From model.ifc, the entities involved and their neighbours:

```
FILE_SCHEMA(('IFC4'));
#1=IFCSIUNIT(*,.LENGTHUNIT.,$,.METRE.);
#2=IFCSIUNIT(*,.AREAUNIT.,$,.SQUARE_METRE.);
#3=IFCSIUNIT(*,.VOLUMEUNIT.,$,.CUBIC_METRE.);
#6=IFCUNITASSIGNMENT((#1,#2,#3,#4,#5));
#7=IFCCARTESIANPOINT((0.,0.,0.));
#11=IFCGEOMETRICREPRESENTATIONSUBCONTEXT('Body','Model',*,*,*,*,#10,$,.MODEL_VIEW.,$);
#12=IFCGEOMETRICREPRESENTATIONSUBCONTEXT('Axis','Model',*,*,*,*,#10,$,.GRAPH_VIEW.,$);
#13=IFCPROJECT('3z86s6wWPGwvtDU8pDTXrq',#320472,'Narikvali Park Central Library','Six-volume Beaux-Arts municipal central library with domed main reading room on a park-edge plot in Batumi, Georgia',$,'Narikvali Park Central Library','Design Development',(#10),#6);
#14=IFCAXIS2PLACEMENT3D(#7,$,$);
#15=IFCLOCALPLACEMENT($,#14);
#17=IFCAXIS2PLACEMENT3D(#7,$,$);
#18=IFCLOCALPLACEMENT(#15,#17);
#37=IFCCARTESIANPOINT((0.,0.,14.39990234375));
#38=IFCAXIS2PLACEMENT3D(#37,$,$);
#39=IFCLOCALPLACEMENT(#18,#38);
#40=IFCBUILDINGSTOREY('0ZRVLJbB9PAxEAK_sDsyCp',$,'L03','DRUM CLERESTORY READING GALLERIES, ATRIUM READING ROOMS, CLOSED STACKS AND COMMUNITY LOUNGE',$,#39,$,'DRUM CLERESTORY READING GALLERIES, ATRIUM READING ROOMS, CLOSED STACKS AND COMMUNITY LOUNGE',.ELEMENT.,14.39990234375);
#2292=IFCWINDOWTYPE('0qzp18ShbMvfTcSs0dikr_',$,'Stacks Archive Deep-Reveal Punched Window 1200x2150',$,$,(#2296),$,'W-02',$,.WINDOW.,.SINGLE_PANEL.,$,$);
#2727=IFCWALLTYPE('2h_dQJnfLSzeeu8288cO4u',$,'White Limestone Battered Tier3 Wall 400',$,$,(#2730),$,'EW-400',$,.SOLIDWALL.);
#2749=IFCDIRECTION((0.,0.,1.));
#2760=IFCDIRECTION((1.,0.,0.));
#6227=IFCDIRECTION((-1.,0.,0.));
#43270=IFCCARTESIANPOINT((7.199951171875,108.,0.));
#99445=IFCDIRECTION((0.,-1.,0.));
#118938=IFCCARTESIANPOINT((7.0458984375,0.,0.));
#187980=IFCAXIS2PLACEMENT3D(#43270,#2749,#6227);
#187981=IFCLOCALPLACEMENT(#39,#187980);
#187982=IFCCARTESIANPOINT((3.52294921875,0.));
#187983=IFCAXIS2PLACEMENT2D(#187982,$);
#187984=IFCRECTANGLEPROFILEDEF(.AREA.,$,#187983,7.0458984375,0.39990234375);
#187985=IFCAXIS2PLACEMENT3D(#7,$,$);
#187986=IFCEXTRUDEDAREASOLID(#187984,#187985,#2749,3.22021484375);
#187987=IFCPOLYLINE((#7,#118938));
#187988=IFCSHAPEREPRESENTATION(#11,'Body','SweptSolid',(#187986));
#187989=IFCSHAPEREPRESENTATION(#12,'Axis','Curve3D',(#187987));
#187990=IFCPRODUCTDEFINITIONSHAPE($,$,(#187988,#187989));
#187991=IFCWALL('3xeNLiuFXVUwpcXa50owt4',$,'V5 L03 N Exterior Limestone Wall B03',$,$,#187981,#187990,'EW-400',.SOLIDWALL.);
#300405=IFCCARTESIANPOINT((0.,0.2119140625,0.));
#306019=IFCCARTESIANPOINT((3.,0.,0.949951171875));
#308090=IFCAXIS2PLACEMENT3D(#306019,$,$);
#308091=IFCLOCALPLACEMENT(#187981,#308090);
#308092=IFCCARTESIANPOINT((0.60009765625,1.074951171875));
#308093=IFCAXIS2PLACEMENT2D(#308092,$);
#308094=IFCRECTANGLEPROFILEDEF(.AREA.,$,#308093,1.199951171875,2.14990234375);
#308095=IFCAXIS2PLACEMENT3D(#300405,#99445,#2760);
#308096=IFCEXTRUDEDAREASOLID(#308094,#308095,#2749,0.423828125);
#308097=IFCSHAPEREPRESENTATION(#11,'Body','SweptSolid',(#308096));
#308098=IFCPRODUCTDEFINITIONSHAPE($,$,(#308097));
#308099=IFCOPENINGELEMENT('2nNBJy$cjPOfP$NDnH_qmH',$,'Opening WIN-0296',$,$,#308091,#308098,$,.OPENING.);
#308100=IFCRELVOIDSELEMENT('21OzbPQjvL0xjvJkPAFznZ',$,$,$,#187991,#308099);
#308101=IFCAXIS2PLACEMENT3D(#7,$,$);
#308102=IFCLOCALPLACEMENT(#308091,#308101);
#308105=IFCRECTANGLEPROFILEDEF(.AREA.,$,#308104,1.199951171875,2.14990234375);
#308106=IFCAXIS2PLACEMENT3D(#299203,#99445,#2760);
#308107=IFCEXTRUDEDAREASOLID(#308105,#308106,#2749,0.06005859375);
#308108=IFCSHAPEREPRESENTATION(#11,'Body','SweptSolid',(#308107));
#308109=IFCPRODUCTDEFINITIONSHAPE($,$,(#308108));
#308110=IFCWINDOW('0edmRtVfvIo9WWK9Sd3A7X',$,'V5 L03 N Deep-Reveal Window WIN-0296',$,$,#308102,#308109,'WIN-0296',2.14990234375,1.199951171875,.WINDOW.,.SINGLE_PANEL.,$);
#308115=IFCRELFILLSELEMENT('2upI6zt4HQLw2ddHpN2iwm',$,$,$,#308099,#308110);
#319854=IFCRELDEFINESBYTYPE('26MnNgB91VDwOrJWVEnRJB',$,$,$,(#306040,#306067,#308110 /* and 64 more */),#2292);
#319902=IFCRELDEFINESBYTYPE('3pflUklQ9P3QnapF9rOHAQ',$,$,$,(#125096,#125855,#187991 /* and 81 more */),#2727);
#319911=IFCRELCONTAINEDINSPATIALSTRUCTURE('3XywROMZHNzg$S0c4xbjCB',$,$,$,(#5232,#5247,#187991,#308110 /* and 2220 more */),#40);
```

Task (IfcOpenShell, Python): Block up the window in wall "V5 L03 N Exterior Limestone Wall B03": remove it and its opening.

```python
import ifcopenshell
import ifcopenshell.api.feature
import ifcopenshell.api.root
import ifcopenshell.geom
import ifcopenshell.util.shape

model = ifcopenshell.open("model.ifc")
settings = ifcopenshell.geom.settings()


def volume(element):
    """Net volume in cubic metres, openings subtracted."""
    shape = ifcopenshell.geom.create_shape(settings, element)
    return ifcopenshell.util.shape.get_volume(shape.geometry)


window = model.by_guid("0edmRtVfvIo9WWK9Sd3A7X")
opening = window.FillsVoids[0].RelatingOpeningElement
wall = opening.VoidsElements[0].RelatingBuildingElement
before = volume(wall)

ifcopenshell.api.root.remove_product(model, product=window)
ifcopenshell.api.feature.remove_feature(model, feature=opening)

after = volume(wall)

print(f"wall volume {before:.3f} -> {after:.3f} m3")

model.write("model-out.ifc")
```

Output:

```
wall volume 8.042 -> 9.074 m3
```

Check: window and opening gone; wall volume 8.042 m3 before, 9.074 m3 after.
